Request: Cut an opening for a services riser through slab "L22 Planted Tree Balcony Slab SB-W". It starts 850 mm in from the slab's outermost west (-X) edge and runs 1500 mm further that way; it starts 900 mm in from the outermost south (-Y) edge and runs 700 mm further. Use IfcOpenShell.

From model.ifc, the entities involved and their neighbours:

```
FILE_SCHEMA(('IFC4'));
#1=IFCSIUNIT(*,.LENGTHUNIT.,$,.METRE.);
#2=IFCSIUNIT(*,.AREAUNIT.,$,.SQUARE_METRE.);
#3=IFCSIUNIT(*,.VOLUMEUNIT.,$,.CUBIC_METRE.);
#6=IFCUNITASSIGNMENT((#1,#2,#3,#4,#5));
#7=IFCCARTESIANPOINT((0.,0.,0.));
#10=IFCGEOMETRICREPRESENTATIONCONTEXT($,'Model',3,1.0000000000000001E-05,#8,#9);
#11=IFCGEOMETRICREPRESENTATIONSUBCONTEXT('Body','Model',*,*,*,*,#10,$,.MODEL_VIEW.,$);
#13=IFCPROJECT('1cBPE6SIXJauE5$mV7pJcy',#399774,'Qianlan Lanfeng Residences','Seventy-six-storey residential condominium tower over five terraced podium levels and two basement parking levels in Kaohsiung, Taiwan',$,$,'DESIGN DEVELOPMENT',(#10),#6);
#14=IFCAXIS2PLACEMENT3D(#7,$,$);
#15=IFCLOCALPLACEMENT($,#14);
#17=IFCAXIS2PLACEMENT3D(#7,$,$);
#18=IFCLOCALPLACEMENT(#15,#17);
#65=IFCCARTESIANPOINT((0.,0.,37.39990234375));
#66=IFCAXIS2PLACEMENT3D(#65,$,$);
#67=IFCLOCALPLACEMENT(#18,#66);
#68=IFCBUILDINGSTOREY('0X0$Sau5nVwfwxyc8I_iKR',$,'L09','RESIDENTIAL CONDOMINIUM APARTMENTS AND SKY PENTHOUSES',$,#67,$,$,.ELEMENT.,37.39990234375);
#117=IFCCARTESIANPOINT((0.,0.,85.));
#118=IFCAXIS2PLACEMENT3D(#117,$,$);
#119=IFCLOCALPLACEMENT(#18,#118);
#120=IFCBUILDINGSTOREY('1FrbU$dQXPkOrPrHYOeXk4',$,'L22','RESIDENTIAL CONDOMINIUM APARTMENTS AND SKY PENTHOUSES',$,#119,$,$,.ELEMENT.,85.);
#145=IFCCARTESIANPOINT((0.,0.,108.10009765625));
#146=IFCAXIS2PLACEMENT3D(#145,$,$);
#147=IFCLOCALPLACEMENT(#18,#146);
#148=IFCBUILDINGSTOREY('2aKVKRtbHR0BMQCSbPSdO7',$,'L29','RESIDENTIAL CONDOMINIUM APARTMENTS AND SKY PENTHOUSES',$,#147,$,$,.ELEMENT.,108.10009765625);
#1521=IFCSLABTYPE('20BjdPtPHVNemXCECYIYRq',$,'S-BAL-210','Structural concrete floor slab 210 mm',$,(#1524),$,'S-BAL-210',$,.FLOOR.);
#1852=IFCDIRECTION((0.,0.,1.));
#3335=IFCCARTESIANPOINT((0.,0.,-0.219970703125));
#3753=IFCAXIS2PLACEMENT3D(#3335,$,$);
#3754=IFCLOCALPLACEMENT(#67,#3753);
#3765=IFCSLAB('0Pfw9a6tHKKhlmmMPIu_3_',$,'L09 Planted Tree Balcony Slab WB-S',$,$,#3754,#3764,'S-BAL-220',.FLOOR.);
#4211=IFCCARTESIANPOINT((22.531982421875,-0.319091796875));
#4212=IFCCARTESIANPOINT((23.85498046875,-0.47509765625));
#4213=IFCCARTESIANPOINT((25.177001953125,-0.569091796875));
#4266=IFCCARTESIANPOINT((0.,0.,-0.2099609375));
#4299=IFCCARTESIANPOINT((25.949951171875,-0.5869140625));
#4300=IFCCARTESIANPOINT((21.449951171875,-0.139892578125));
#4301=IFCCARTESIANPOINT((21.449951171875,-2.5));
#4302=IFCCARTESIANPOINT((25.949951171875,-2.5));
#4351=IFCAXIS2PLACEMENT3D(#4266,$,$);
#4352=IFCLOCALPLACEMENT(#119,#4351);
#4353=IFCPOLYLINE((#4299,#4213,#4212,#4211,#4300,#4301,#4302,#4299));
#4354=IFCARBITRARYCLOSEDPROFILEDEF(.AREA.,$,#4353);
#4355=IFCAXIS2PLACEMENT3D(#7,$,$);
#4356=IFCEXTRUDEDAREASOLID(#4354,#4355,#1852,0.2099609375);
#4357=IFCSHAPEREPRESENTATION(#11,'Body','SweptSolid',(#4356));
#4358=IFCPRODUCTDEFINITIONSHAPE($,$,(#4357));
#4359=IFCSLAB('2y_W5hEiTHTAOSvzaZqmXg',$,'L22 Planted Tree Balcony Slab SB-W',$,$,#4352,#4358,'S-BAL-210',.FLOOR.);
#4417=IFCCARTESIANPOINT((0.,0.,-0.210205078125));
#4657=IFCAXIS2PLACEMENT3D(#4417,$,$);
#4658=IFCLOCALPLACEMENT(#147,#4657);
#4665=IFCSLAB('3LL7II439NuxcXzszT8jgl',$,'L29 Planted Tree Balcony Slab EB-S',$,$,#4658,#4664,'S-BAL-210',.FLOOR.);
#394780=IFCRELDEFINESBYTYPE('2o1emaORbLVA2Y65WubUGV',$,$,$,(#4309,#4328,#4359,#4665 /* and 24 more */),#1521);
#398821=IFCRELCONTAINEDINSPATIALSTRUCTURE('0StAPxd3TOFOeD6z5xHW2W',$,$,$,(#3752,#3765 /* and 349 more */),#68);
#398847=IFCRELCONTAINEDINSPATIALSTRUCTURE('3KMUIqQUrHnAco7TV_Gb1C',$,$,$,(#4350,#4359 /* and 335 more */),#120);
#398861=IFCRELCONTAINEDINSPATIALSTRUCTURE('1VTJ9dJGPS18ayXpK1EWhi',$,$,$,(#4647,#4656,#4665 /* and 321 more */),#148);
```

```python
import numpy as np
import ifcopenshell
import ifcopenshell.api.feature
import ifcopenshell.api.geometry
import ifcopenshell.api.root
import ifcopenshell.geom
import ifcopenshell.util.placement
import ifcopenshell.util.representation
import ifcopenshell.util.shape
import ifcopenshell.util.unit

model = ifcopenshell.open("model.ifc")
unit_scale = ifcopenshell.util.unit.calculate_unit_scale(model)
settings = ifcopenshell.geom.settings()


def volume(element):
    """Net volume in cubic metres, openings subtracted."""
    shape = ifcopenshell.geom.create_shape(settings, element)
    return ifcopenshell.util.shape.get_volume(shape.geometry)


slab = model.by_guid("2y_W5hEiTHTAOSvzaZqmXg")
before = volume(slab)

# Extent in the slab's own axes, in metres. The edges named are its -X and -Y sides.
slab_shape = ifcopenshell.geom.create_shape(settings, slab)
vertices = ifcopenshell.util.shape.get_vertices(slab_shape.geometry)
x_min, y_min, bottom = vertices.min(axis=0)
top = vertices[:, 2].max()

opening = ifcopenshell.api.root.create_entity(model, ifc_class="IfcOpeningElement", name="Services riser opening", predefined_type="OPENING")
context = ifcopenshell.util.representation.get_context(model, "Model", "Body", "MODEL_VIEW")
width, depth = 1.5, 0.7
outline = [(0.0, 0.0), (width, 0.0), (width, depth), (0.0, depth), (0.0, 0.0)]
# Overshoot both faces by 50 mm so the cut is clean.
shape = ifcopenshell.api.geometry.add_slab_representation(
    model, context=context, depth=top - bottom + 0.1, polyline=outline
)
ifcopenshell.api.geometry.assign_representation(model, product=opening, representation=shape)

matrix = ifcopenshell.util.placement.get_local_placement(slab.ObjectPlacement)
matrix[:, 3] = matrix @ np.append(np.array([x_min + 0.85, y_min + 0.9, bottom - 0.05]) / unit_scale, 1.0)
ifcopenshell.api.geometry.edit_object_placement(model, product=opening, matrix=matrix, is_si=False)
ifcopenshell.api.feature.add_feature(model, feature=opening, element=slab)

after = volume(slab)

print(f"slab volume {before:.3f} -> {after:.3f} m3")

model.write("model_v2.ifc")
```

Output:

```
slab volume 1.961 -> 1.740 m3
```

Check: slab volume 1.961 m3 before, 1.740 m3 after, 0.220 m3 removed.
